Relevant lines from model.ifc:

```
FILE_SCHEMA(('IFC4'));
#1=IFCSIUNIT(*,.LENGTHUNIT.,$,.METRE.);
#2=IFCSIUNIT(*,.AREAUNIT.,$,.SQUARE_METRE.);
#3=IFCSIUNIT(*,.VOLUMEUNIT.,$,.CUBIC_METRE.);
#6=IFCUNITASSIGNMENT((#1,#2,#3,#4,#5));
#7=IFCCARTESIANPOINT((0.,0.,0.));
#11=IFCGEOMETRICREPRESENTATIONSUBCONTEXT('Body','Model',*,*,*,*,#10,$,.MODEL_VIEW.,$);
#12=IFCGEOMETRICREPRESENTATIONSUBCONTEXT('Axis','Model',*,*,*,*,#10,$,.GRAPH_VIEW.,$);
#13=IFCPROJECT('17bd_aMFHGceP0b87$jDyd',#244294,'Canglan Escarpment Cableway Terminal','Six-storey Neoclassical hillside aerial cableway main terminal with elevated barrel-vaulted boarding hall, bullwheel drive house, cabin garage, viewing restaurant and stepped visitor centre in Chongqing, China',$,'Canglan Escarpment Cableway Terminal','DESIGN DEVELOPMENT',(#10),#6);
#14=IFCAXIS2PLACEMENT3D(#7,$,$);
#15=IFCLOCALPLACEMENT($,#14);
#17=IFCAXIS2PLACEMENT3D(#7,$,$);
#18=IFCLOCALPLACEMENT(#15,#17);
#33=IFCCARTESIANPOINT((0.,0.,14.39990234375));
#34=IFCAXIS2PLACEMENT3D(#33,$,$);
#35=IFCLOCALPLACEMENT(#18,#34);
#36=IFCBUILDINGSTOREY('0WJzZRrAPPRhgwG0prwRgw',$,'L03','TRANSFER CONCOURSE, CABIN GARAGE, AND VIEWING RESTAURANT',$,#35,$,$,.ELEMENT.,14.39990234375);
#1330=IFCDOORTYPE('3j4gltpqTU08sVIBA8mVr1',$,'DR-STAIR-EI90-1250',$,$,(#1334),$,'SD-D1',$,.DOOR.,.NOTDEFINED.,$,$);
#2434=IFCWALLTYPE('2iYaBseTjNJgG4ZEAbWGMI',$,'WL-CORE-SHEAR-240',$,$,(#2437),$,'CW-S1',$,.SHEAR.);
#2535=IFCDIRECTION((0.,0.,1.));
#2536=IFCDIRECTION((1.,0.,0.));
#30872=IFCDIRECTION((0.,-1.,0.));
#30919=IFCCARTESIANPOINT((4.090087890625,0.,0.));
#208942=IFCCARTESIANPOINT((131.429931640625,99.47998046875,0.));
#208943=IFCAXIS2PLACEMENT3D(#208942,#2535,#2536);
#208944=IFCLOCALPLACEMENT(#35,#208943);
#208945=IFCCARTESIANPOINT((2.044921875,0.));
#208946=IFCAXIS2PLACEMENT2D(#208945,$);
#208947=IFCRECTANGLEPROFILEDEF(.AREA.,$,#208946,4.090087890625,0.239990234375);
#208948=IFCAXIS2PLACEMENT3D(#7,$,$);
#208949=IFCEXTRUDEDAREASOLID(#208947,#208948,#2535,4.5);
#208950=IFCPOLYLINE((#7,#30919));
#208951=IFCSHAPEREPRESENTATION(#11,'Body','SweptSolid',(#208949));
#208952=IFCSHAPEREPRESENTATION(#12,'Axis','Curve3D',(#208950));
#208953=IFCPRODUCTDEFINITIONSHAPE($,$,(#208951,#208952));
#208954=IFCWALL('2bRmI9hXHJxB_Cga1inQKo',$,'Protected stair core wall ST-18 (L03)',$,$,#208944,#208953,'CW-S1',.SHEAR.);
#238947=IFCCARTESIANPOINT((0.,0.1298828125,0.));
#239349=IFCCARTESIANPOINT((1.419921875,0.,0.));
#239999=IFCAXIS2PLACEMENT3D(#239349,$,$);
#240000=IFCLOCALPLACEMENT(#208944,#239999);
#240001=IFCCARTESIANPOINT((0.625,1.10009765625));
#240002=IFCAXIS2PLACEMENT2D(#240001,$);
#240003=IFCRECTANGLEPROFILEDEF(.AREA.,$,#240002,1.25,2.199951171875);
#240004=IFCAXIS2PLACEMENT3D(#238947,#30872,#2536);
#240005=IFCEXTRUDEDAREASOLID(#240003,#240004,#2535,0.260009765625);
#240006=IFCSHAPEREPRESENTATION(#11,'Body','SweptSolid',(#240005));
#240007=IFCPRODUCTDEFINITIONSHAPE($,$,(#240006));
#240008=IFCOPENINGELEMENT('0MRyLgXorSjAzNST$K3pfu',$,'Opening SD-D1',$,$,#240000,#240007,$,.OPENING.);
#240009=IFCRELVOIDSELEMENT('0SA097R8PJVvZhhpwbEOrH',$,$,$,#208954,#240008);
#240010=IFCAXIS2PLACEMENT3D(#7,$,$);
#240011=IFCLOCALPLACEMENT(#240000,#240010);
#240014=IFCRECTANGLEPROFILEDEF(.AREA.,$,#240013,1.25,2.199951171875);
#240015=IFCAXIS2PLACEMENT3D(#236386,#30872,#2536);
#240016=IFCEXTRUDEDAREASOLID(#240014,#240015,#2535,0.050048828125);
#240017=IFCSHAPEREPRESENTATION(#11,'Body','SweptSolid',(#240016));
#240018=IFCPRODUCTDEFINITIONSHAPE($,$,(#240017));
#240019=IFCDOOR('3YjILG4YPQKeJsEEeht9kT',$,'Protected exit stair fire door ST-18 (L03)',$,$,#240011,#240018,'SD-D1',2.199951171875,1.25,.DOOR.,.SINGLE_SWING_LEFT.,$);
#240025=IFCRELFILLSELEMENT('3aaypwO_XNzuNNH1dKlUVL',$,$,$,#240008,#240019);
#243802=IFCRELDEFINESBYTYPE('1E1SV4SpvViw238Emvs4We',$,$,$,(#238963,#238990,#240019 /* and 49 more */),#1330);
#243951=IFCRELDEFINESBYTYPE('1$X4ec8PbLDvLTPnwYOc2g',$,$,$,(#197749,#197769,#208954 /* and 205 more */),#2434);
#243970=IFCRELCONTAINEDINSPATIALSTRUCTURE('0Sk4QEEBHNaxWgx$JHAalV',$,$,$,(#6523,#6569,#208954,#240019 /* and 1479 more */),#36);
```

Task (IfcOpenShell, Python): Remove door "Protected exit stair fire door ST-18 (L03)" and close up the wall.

```python
import ifcopenshell
import ifcopenshell.api.feature
import ifcopenshell.api.root
import ifcopenshell.geom
import ifcopenshell.util.shape

model = ifcopenshell.open("model.ifc")
settings = ifcopenshell.geom.settings()


def volume(element):
    """Net volume in cubic metres, openings subtracted."""
    shape = ifcopenshell.geom.create_shape(settings, element)
    return ifcopenshell.util.shape.get_volume(shape.geometry)


door = model.by_guid("3YjILG4YPQKeJsEEeht9kT")
opening = door.FillsVoids[0].RelatingOpeningElement
wall = opening.VoidsElements[0].RelatingBuildingElement
before = volume(wall)

ifcopenshell.api.root.remove_product(model, product=door)
ifcopenshell.api.feature.remove_feature(model, feature=opening)

after = volume(wall)

print(f"wall volume {before:.3f} -> {after:.3f} m3")

model.write("model_edited.ifc")
```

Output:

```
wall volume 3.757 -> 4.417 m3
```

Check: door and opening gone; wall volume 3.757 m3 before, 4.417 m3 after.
